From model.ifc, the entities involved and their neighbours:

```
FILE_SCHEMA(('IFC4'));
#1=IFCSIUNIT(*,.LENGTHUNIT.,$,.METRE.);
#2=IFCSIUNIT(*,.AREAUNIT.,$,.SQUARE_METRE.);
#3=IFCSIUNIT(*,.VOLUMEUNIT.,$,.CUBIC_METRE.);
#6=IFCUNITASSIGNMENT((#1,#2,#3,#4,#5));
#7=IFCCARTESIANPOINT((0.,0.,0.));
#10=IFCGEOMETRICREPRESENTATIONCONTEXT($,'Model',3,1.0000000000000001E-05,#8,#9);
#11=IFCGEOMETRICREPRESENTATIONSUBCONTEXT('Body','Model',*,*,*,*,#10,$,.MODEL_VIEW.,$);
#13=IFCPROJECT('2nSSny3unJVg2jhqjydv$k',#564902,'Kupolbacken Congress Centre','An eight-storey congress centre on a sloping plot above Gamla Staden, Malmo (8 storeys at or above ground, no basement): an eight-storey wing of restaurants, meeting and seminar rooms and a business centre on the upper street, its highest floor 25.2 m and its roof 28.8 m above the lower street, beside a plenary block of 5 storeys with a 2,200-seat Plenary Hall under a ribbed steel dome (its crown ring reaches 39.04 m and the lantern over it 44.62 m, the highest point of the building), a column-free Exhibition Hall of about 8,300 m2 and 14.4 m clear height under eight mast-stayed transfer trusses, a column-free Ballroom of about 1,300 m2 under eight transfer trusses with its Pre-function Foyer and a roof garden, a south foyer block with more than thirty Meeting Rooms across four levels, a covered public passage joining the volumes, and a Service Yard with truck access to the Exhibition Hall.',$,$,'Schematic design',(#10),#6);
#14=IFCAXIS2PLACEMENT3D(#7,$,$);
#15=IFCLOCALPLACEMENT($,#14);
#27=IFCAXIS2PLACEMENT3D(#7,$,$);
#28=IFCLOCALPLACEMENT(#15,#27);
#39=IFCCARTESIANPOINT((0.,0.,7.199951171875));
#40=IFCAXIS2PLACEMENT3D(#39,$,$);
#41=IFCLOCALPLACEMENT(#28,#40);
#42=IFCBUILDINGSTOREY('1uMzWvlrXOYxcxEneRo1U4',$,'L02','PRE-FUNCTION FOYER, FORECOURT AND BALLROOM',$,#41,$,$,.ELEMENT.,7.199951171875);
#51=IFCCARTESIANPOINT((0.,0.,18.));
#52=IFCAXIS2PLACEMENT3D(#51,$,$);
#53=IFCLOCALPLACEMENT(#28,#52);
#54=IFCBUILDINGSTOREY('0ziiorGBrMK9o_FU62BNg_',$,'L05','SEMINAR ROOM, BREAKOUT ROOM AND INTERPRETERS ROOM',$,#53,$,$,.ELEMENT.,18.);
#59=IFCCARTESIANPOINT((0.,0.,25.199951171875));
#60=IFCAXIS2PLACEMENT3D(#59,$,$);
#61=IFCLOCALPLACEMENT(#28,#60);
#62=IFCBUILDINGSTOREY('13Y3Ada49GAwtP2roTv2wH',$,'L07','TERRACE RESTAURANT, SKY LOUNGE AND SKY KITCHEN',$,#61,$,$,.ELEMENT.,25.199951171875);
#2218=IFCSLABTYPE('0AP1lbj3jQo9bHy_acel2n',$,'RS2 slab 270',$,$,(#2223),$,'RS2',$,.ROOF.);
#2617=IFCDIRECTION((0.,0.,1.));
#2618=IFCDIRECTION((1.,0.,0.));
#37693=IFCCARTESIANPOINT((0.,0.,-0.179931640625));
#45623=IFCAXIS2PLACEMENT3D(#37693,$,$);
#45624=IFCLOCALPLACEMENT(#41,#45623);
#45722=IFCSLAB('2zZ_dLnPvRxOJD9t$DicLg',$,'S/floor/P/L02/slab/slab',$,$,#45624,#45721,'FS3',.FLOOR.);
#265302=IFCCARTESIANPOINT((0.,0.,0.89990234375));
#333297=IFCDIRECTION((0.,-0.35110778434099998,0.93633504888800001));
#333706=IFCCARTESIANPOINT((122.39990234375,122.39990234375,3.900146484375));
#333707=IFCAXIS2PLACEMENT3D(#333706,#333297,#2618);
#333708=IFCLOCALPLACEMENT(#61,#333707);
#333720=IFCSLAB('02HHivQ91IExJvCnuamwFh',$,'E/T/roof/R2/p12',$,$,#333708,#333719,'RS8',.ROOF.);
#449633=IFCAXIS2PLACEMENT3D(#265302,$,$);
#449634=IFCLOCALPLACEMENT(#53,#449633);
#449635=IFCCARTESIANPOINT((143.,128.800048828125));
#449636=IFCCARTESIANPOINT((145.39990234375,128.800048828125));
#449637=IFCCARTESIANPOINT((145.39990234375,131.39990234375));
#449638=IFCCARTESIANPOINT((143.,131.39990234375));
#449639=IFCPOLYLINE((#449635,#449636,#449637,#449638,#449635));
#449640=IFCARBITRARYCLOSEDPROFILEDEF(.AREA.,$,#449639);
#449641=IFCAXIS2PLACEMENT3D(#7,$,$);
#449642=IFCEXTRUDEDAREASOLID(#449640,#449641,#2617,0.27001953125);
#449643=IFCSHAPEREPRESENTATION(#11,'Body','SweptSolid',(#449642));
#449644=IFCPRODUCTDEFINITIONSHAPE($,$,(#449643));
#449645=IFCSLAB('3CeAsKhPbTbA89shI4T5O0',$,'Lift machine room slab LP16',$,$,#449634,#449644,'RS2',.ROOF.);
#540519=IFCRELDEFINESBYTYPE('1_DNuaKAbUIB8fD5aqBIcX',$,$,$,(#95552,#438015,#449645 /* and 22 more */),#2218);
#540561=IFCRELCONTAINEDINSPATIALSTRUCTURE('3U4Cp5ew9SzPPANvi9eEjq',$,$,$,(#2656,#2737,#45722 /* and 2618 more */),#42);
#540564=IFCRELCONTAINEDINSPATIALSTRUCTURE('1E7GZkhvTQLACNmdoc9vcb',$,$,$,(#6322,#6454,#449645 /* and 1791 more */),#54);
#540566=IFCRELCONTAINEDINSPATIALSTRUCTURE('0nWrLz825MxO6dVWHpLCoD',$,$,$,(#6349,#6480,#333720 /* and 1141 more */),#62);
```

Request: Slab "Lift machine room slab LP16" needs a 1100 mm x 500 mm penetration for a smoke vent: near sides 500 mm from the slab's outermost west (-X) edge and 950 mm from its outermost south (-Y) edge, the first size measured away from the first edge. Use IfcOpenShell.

```python
import numpy as np
import ifcopenshell
import ifcopenshell.api.feature
import ifcopenshell.api.geometry
import ifcopenshell.api.root
import ifcopenshell.geom
import ifcopenshell.util.placement
import ifcopenshell.util.representation
import ifcopenshell.util.shape
import ifcopenshell.util.unit

model = ifcopenshell.open("model.ifc")
unit_scale = ifcopenshell.util.unit.calculate_unit_scale(model)
settings = ifcopenshell.geom.settings()


def volume(element):
    """Net volume in cubic metres, openings subtracted."""
    shape = ifcopenshell.geom.create_shape(settings, element)
    return ifcopenshell.util.shape.get_volume(shape.geometry)


slab = model.by_guid("3CeAsKhPbTbA89shI4T5O0")
before = volume(slab)

# Extent in the slab's own axes, in metres. The edges named are its -X and -Y sides.
slab_shape = ifcopenshell.geom.create_shape(settings, slab)
vertices = ifcopenshell.util.shape.get_vertices(slab_shape.geometry)
x_min, y_min, bottom = vertices.min(axis=0)
top = vertices[:, 2].max()

opening = ifcopenshell.api.root.create_entity(model, ifc_class="IfcOpeningElement", name="Smoke vent opening", predefined_type="OPENING")
context = ifcopenshell.util.representation.get_context(model, "Model", "Body", "MODEL_VIEW")
width, depth = 1.1, 0.5
outline = [(0.0, 0.0), (width, 0.0), (width, depth), (0.0, depth), (0.0, 0.0)]
# Overshoot both faces by 50 mm so the cut is clean.
shape = ifcopenshell.api.geometry.add_slab_representation(
    model, context=context, depth=top - bottom + 0.1, polyline=outline
)
ifcopenshell.api.geometry.assign_representation(model, product=opening, representation=shape)

matrix = ifcopenshell.util.placement.get_local_placement(slab.ObjectPlacement)
matrix[:, 3] = matrix @ np.append(np.array([x_min + 0.5, y_min + 0.95, bottom - 0.05]) / unit_scale, 1.0)
ifcopenshell.api.geometry.edit_object_placement(model, product=opening, matrix=matrix, is_si=False)
ifcopenshell.api.feature.add_feature(model, feature=opening, element=slab)

after = volume(slab)

print(f"slab volume {before:.3f} -> {after:.3f} m3")

model.write("model_v2.ifc")
```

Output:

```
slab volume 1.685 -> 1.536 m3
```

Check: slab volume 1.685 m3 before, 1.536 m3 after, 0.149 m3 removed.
